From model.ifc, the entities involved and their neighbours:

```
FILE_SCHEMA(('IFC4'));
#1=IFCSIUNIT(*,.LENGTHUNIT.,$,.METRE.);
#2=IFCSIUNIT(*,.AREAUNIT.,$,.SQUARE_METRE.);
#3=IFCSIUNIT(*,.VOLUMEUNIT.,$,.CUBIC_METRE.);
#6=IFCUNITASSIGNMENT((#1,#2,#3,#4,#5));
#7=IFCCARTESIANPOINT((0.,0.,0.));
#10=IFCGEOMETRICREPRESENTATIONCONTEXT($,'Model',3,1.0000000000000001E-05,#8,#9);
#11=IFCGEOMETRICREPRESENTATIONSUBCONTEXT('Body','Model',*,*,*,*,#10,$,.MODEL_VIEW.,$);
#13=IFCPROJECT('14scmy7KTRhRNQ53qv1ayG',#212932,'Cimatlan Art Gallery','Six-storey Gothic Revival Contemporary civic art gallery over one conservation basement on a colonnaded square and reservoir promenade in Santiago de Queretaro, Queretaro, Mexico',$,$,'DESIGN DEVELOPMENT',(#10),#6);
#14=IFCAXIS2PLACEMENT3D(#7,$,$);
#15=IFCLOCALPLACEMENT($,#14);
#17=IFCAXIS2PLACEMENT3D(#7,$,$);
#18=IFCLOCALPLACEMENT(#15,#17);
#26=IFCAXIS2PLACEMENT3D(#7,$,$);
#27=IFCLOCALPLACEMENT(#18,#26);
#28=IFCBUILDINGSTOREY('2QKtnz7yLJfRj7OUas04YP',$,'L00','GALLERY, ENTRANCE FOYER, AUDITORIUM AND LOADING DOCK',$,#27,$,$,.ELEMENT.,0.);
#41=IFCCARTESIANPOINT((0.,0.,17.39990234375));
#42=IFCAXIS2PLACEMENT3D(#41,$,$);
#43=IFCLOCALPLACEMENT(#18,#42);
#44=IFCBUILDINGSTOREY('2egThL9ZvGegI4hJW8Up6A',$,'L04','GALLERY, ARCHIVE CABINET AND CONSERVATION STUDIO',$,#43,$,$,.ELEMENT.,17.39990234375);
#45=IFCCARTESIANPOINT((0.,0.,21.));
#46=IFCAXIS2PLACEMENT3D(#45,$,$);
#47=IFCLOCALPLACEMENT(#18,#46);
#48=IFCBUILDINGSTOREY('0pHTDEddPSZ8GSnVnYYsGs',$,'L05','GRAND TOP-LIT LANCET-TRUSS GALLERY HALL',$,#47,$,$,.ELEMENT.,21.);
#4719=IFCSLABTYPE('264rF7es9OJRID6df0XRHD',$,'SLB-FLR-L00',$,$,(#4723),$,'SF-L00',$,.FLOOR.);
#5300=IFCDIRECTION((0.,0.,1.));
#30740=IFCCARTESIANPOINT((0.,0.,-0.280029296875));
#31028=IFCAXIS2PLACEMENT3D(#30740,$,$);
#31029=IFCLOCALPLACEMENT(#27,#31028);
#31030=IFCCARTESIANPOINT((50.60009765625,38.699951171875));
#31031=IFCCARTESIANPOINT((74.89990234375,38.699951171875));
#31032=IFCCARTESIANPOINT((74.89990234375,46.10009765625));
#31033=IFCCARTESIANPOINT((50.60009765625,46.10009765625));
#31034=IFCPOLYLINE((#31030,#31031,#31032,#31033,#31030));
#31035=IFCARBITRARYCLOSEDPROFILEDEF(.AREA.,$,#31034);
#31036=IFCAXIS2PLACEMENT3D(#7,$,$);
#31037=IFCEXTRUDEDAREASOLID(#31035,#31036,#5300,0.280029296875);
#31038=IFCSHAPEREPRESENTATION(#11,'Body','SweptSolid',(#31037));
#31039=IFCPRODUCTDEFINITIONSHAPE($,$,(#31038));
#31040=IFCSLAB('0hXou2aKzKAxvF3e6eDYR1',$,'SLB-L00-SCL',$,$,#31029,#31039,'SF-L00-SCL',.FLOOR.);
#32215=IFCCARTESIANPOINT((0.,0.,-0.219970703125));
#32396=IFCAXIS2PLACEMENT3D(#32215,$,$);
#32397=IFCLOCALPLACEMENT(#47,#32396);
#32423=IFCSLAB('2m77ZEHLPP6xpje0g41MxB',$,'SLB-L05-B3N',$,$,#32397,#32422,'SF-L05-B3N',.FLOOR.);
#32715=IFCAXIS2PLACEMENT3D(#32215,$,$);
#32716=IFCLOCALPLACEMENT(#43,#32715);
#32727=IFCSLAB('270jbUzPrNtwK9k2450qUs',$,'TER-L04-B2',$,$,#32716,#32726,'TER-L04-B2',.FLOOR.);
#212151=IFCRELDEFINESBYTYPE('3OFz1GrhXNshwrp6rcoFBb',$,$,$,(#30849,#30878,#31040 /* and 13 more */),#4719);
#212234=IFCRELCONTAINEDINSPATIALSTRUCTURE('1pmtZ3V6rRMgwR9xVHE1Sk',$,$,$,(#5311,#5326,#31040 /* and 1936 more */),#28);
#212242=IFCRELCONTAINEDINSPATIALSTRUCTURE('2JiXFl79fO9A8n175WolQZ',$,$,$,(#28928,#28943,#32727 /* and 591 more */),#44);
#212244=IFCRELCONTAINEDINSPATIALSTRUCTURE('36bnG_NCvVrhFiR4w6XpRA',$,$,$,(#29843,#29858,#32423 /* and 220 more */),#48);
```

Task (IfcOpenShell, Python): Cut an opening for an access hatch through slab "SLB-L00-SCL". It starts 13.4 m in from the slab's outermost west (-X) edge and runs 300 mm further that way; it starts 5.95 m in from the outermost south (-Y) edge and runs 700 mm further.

```python
import numpy as np
import ifcopenshell
import ifcopenshell.api.feature
import ifcopenshell.api.geometry
import ifcopenshell.api.root
import ifcopenshell.geom
import ifcopenshell.util.placement
import ifcopenshell.util.representation
import ifcopenshell.util.shape
import ifcopenshell.util.unit

model = ifcopenshell.open("model.ifc")
unit_scale = ifcopenshell.util.unit.calculate_unit_scale(model)
settings = ifcopenshell.geom.settings()


def volume(element):
    """Net volume in cubic metres, openings subtracted."""
    shape = ifcopenshell.geom.create_shape(settings, element)
    return ifcopenshell.util.shape.get_volume(shape.geometry)


slab = model.by_id(31040)
before = volume(slab)

# Extent in the slab's own axes, in metres. The edges named are its -X and -Y sides.
slab_shape = ifcopenshell.geom.create_shape(settings, slab)
vertices = ifcopenshell.util.shape.get_vertices(slab_shape.geometry)
x_min, y_min, bottom = vertices.min(axis=0)
top = vertices[:, 2].max()

opening = ifcopenshell.api.root.create_entity(model, ifc_class="IfcOpeningElement", name="Access hatch opening", predefined_type="OPENING")
context = ifcopenshell.util.representation.get_context(model, "Model", "Body", "MODEL_VIEW")
width, depth = 0.3, 0.7
outline = [(0.0, 0.0), (width, 0.0), (width, depth), (0.0, depth), (0.0, 0.0)]
# Overshoot both faces by 50 mm so the cut is clean.
shape = ifcopenshell.api.geometry.add_slab_representation(
    model, context=context, depth=top - bottom + 0.1, polyline=outline
)
ifcopenshell.api.geometry.assign_representation(model, product=opening, representation=shape)

matrix = ifcopenshell.util.placement.get_local_placement(slab.ObjectPlacement)
matrix[:, 3] = matrix @ np.append(np.array([x_min + 13.4, y_min + 5.95, bottom - 0.05]) / unit_scale, 1.0)
ifcopenshell.api.geometry.edit_object_placement(model, product=opening, matrix=matrix, is_si=False)
ifcopenshell.api.feature.add_feature(model, feature=opening, element=slab)

after = volume(slab)

print(f"slab volume {before:.3f} -> {after:.3f} m3")

model.write("model_edited.ifc")
```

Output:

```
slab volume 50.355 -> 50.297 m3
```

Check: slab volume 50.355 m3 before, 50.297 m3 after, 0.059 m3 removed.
